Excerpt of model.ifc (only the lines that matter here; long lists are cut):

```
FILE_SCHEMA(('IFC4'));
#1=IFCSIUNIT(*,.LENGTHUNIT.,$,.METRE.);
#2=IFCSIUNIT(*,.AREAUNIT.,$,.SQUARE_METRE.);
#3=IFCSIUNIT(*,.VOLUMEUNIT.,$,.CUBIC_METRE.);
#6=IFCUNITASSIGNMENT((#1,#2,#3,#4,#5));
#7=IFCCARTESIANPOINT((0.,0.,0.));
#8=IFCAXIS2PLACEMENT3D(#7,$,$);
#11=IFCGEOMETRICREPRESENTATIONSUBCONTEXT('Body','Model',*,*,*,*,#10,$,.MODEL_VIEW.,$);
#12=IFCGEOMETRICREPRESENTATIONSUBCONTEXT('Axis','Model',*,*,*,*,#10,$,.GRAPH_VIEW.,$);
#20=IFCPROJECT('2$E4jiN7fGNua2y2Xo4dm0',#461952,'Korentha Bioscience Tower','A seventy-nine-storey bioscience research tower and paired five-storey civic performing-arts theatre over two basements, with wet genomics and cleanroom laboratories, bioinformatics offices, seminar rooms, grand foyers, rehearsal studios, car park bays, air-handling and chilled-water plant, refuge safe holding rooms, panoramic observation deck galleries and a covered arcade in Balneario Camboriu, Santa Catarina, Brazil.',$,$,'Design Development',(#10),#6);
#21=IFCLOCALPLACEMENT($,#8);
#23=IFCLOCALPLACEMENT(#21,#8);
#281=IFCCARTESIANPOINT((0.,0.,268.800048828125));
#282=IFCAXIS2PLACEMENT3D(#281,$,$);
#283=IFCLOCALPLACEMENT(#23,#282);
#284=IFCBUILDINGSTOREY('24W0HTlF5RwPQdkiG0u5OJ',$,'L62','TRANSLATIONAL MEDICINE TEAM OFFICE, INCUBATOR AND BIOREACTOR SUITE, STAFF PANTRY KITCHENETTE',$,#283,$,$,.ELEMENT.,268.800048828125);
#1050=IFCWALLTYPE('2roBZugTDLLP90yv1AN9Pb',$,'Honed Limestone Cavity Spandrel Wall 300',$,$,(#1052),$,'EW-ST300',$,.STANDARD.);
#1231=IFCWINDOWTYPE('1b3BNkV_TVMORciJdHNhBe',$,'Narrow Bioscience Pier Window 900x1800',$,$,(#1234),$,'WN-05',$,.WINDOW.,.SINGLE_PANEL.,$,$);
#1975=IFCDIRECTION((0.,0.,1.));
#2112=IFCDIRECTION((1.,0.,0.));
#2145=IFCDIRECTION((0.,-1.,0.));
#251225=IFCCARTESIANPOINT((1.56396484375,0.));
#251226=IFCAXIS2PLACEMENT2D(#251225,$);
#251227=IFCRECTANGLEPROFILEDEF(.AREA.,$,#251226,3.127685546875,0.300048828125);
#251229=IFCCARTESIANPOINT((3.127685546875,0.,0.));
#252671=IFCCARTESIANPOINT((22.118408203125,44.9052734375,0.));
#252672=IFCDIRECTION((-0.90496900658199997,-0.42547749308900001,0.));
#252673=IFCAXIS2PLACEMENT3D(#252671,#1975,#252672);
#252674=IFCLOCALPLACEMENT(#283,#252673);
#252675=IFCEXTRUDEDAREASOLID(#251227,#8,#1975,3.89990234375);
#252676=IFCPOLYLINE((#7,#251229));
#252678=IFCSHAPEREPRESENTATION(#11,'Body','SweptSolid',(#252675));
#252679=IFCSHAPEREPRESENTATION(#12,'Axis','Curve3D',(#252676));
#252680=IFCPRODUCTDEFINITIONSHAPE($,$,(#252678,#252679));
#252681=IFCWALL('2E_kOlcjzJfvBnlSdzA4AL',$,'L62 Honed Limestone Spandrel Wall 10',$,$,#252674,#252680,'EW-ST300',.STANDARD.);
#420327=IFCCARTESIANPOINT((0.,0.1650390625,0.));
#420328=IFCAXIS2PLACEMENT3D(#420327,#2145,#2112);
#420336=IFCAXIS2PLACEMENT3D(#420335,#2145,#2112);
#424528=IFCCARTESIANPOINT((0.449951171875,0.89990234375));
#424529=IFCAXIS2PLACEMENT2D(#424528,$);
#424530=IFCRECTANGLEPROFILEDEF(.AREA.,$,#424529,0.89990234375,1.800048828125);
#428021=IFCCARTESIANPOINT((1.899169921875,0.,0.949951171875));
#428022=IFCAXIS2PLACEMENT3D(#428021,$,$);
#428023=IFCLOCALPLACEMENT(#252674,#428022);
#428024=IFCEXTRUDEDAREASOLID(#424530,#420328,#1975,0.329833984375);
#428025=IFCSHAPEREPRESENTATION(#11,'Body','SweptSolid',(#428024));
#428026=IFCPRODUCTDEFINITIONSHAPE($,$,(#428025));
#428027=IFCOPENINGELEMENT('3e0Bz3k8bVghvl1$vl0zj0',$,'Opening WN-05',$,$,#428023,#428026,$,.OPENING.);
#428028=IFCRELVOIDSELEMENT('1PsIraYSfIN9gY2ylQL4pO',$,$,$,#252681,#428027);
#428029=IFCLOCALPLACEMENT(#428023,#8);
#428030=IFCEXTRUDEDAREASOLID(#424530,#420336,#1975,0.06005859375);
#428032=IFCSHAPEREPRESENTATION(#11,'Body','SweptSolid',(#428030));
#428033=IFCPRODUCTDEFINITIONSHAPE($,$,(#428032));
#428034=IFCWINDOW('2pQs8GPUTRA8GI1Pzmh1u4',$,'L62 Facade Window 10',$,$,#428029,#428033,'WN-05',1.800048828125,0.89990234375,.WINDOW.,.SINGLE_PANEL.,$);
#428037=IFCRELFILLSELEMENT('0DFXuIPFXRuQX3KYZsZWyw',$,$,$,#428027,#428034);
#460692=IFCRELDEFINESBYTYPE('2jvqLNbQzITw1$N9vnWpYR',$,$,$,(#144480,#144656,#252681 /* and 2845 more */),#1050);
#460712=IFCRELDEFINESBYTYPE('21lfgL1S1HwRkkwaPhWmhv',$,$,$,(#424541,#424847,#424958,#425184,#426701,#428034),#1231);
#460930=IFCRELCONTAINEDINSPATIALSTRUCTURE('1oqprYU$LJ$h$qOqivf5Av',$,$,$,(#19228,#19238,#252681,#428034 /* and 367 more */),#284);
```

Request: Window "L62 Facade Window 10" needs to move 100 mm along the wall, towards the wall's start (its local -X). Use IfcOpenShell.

```python
import ifcopenshell
import ifcopenshell.api.geometry
import ifcopenshell.util.placement

model = ifcopenshell.open("model.ifc")

window = model.by_guid("2pQs8GPUTRA8GI1Pzmh1u4")
opening = window.FillsVoids[0].RelatingOpeningElement
wall = opening.VoidsElements[0].RelatingBuildingElement

wall_matrix = ifcopenshell.util.placement.get_local_placement(wall.ObjectPlacement)
shift = wall_matrix[:3, 0] * -0.1
before = ifcopenshell.util.placement.get_local_placement(window.ObjectPlacement)[:3, 3].copy()

# The window is placed relative to its opening, so it follows when the opening moves.
matrix = ifcopenshell.util.placement.get_local_placement(opening.ObjectPlacement)
matrix[:3, 3] += shift
ifcopenshell.api.geometry.edit_object_placement(
    model, product=opening, matrix=matrix, is_si=False, should_transform_children=True
)

after = ifcopenshell.util.placement.get_local_placement(window.ObjectPlacement)[:3, 3]
print("window moved by", (after - before).round(3) + 0.0)

model.write("model-out.ifc")
```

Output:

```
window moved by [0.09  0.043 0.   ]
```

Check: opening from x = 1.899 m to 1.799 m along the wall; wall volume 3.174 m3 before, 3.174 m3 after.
